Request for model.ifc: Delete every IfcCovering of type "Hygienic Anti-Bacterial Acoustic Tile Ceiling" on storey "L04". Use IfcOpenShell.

First a look at what the model holds.

```python
import ifcopenshell
import ifcopenshell.util.element

model = ifcopenshell.open("model.ifc")
print(model.schema)
storey = next(s for s in model.by_type("IfcBuildingStorey") if s.Name == "L04")
coverings = [e for e in ifcopenshell.util.element.get_decomposition(storey) if e.is_a("IfcCovering")]
seen = {}
for e in coverings:
    element_type = ifcopenshell.util.element.get_type(e)
    name = element_type.Name if element_type not in (None, e) else None
    seen[name] = seen.get(name, 0) + 1
for name, count in sorted(seen.items(), key=str):
    print(count, "x", name)
```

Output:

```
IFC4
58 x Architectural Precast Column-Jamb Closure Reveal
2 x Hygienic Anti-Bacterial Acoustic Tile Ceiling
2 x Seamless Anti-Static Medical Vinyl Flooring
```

```python
import ifcopenshell
import ifcopenshell.api.root
import ifcopenshell.util.element

model = ifcopenshell.open("model.ifc")

storey = next(s for s in model.by_type("IfcBuildingStorey") if s.Name == "L04")
coverings = [e for e in ifcopenshell.util.element.get_decomposition(storey) if e.is_a("IfcCovering")]
targets = [e for e in coverings if (t := ifcopenshell.util.element.get_type(e)) not in (None, e) and t.Name == "Hygienic Anti-Bacterial Acoustic Tile Ceiling"]

for e in targets:
    ifcopenshell.api.root.remove_product(model, product=e)
print(len(targets), "removed")

model.write("model_edited.ifc")
```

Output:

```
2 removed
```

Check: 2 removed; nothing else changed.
